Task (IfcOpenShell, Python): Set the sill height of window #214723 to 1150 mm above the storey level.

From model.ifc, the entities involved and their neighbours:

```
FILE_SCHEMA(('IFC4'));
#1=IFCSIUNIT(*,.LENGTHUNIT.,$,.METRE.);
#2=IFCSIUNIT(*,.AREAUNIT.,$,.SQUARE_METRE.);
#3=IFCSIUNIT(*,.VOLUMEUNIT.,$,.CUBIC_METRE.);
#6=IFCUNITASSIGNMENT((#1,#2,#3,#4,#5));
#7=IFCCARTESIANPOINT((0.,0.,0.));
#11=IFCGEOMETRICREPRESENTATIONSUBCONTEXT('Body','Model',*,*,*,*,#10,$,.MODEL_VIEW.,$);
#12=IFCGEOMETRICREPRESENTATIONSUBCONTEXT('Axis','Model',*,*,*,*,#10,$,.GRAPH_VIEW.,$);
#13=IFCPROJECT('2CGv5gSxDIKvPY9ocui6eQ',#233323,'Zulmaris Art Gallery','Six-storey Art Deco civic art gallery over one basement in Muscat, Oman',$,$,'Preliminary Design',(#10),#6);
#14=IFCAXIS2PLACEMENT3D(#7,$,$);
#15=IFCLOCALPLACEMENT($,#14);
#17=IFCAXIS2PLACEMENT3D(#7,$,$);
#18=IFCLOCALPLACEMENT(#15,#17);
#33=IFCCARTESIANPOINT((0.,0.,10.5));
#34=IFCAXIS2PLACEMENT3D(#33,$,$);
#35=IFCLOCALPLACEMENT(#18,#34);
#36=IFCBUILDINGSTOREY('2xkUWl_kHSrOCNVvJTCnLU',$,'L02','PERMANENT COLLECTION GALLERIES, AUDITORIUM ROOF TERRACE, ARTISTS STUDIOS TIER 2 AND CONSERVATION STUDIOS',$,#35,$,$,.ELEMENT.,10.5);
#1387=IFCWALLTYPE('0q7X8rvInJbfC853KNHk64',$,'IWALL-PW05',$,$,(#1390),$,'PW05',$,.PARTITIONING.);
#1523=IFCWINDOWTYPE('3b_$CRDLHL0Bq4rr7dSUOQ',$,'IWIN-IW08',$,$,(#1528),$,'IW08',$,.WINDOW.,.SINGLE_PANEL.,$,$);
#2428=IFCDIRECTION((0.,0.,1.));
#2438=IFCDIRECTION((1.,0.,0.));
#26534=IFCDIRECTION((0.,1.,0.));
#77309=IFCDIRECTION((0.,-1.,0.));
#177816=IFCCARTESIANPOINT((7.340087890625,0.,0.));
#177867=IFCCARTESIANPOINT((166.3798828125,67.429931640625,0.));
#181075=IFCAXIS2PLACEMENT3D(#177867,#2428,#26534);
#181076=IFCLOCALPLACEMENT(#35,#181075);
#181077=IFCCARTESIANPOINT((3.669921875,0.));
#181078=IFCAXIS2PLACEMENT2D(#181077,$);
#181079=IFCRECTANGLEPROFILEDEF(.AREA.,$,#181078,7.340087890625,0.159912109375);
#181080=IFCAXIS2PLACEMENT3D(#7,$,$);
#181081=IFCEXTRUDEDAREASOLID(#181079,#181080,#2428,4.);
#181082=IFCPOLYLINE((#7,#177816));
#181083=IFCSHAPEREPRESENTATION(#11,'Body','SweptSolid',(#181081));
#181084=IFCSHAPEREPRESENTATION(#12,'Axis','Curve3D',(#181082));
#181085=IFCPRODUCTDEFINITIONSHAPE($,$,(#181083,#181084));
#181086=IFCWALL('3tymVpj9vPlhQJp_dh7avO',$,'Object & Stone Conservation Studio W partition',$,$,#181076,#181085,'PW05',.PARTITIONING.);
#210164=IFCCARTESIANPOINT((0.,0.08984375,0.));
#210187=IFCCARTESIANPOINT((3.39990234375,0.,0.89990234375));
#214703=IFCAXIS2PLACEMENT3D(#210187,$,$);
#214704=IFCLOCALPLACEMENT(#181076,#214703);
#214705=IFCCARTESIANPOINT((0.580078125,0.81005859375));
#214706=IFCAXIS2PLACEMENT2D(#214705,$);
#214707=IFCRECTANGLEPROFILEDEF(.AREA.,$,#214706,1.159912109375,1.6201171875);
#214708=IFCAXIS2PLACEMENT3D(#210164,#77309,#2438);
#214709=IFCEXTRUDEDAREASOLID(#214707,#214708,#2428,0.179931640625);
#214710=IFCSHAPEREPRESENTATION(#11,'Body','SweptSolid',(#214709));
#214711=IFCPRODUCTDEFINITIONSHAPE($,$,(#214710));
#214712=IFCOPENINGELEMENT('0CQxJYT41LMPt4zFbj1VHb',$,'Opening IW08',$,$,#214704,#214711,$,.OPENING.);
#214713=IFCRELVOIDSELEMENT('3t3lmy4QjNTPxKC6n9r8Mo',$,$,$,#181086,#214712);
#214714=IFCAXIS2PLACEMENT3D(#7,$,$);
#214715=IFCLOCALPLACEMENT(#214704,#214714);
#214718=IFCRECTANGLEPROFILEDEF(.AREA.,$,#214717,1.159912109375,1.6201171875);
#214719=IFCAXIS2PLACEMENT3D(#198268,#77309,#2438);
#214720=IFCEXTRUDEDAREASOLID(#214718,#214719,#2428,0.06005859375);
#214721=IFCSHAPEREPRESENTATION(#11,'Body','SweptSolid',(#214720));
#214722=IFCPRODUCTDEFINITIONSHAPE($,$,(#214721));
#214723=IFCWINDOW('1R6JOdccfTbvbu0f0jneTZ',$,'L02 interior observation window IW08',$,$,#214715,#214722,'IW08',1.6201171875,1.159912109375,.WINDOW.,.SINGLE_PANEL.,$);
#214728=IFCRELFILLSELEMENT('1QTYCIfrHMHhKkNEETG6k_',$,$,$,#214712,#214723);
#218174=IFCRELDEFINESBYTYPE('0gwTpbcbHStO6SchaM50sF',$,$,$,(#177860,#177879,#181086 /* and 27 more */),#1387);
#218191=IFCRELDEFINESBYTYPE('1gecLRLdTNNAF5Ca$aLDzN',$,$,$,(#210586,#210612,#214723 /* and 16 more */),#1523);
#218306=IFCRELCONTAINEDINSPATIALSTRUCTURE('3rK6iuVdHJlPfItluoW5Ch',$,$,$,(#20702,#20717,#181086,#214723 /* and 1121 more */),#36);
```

```python
import numpy as np
import ifcopenshell
import ifcopenshell.api.geometry
import ifcopenshell.geom
import ifcopenshell.util.element
import ifcopenshell.util.placement
import ifcopenshell.util.shape
import ifcopenshell.util.unit

model = ifcopenshell.open("model.ifc")
unit_scale = ifcopenshell.util.unit.calculate_unit_scale(model)

window = model.by_guid("1R6JOdccfTbvbu0f0jneTZ")
opening = window.FillsVoids[0].RelatingOpeningElement
storey = ifcopenshell.util.element.get_container(window, ifc_class="IfcBuildingStorey")
level = ifcopenshell.util.placement.get_local_placement(storey.ObjectPlacement)[2, 3]

# The opening's origin need not be at the sill, so measure its lowest point.
shape = ifcopenshell.geom.create_shape(ifcopenshell.geom.settings(), opening)
bottom = ifcopenshell.util.shape.get_shape_bottom_elevation(shape, shape.geometry) / unit_scale
dz = level + 1.15 - bottom

shift = np.array([0.0, 0.0, dz])
# The window is placed relative to its opening, so it follows when the opening moves.
matrix = ifcopenshell.util.placement.get_local_placement(opening.ObjectPlacement)
matrix[:3, 3] += shift
ifcopenshell.api.geometry.edit_object_placement(
    model, product=opening, matrix=matrix, is_si=False, should_transform_children=True
)

print(f"moved by {dz * unit_scale:+.3f} m")

model.write("model_updated.ifc")
```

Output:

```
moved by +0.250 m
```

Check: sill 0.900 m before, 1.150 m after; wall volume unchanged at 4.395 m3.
